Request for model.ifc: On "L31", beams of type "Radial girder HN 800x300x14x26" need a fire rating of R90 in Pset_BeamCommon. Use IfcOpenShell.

First a look at what the model holds.

```python
import ifcopenshell
import ifcopenshell.util.element

model = ifcopenshell.open("model.ifc")
print(model.schema)
storey = next(s for s in model.by_type("IfcBuildingStorey") if s.Name == "L31")
beams = [e for e in ifcopenshell.util.element.get_decomposition(storey) if e.is_a("IfcBeam")]
seen = {}
for e in beams:
    element_type = ifcopenshell.util.element.get_type(e)
    key = (element_type.Name if element_type != e and element_type else None, ifcopenshell.util.element.get_pset(e, "Pset_BeamCommon", "FireRating"))
    seen[key] = seen.get(key, 0) + 1
for (name, value), count in sorted(seen.items(), key=str):
    print(count, "x", name, "|", value)
```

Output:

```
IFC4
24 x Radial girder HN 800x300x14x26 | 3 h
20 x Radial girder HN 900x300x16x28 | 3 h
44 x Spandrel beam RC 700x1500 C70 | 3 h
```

```python
import ifcopenshell
import ifcopenshell.api.pset
import ifcopenshell.util.element

model = ifcopenshell.open("model.ifc")

storey = next(s for s in model.by_type("IfcBuildingStorey") if s.Name == "L31")
beams = [e for e in ifcopenshell.util.element.get_decomposition(storey) if e.is_a("IfcBeam")]

count = 0
for e in beams:
    element_type = ifcopenshell.util.element.get_type(e)
    if element_type in (None, e) or element_type.Name != "Radial girder HN 800x300x14x26":
        continue
    found = ifcopenshell.util.element.get_pset(e, "Pset_BeamCommon", should_inherit=False)
    if found:
        pset = model.by_id(found["id"])
        if len(ifcopenshell.util.element.get_elements_by_pset(pset)) > 1:
            pset = ifcopenshell.api.pset.unshare_pset(model, products=[e], pset=pset)[0]
    else:
        pset = ifcopenshell.api.pset.add_pset(model, product=e, name="Pset_BeamCommon")
    ifcopenshell.api.pset.edit_pset(model, pset=pset, properties={"FireRating": "R90"})
    count += 1

print(count, "beams updated")

model.write("model_v2.ifc")
```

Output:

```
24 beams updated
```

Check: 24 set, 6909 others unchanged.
